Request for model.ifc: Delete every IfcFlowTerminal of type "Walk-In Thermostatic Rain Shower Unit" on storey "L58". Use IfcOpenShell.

First a look at what the model holds.

```python
import ifcopenshell
import ifcopenshell.util.element

model = ifcopenshell.open("model.ifc")
print(model.schema)
storey = next(s for s in model.by_type("IfcBuildingStorey") if s.Name == "L58")
terminals = [e for e in ifcopenshell.util.element.get_decomposition(storey) if e.is_a("IfcFlowTerminal")]
seen = {}
for e in terminals:
    element_type = ifcopenshell.util.element.get_type(e)
    name = element_type.Name if element_type not in (None, e) else None
    seen[name] = seen.get(name, 0) + 1
for name, count in sorted(seen.items(), key=str):
    print(count, "x", name)
```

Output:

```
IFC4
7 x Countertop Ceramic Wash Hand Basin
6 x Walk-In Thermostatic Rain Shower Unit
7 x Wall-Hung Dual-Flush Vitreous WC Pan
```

```python
import ifcopenshell
import ifcopenshell.api.root
import ifcopenshell.util.element

model = ifcopenshell.open("model.ifc")

storey = next(s for s in model.by_type("IfcBuildingStorey") if s.Name == "L58")
terminals = [e for e in ifcopenshell.util.element.get_decomposition(storey) if e.is_a("IfcFlowTerminal")]
targets = [e for e in terminals if (t := ifcopenshell.util.element.get_type(e)) not in (None, e) and t.Name == "Walk-In Thermostatic Rain Shower Unit"]

for e in targets:
    ifcopenshell.api.root.remove_product(model, product=e)
print(len(targets), "removed")

model.write("model-out.ifc")
```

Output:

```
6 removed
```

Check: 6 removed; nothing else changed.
